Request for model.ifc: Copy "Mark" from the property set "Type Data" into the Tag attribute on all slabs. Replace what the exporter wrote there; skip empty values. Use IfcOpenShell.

First a look at what the model holds.

```python
import ifcopenshell
import ifcopenshell.util.element

model = ifcopenshell.open("model.ifc")
print(model.schema)
slabs = model.by_type("IfcSlab")
print(len(slabs), "slabs")
for e in slabs[:8]:
    source = ifcopenshell.util.element.get_pset(e, "Type Data", "Mark")
    target = e.Tag
    print(e.id(), repr(source), repr(target), sep=" | ")
```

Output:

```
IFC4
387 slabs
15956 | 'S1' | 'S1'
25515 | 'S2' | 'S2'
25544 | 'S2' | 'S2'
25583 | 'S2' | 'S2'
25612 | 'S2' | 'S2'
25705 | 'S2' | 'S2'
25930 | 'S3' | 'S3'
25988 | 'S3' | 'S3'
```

```python
import ifcopenshell
import ifcopenshell.util.element

model = ifcopenshell.open("model.ifc")

count = 0
for e in model.by_type("IfcSlab"):
    value = ifcopenshell.util.element.get_pset(e, "Type Data", "Mark")
    current = e.Tag
    if not value or not value.strip() or current == value:
        continue
    e.Tag = value
    count += 1

print(count, "slabs updated")

model.write("model_v2.ifc")
```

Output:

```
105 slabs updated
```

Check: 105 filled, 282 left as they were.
